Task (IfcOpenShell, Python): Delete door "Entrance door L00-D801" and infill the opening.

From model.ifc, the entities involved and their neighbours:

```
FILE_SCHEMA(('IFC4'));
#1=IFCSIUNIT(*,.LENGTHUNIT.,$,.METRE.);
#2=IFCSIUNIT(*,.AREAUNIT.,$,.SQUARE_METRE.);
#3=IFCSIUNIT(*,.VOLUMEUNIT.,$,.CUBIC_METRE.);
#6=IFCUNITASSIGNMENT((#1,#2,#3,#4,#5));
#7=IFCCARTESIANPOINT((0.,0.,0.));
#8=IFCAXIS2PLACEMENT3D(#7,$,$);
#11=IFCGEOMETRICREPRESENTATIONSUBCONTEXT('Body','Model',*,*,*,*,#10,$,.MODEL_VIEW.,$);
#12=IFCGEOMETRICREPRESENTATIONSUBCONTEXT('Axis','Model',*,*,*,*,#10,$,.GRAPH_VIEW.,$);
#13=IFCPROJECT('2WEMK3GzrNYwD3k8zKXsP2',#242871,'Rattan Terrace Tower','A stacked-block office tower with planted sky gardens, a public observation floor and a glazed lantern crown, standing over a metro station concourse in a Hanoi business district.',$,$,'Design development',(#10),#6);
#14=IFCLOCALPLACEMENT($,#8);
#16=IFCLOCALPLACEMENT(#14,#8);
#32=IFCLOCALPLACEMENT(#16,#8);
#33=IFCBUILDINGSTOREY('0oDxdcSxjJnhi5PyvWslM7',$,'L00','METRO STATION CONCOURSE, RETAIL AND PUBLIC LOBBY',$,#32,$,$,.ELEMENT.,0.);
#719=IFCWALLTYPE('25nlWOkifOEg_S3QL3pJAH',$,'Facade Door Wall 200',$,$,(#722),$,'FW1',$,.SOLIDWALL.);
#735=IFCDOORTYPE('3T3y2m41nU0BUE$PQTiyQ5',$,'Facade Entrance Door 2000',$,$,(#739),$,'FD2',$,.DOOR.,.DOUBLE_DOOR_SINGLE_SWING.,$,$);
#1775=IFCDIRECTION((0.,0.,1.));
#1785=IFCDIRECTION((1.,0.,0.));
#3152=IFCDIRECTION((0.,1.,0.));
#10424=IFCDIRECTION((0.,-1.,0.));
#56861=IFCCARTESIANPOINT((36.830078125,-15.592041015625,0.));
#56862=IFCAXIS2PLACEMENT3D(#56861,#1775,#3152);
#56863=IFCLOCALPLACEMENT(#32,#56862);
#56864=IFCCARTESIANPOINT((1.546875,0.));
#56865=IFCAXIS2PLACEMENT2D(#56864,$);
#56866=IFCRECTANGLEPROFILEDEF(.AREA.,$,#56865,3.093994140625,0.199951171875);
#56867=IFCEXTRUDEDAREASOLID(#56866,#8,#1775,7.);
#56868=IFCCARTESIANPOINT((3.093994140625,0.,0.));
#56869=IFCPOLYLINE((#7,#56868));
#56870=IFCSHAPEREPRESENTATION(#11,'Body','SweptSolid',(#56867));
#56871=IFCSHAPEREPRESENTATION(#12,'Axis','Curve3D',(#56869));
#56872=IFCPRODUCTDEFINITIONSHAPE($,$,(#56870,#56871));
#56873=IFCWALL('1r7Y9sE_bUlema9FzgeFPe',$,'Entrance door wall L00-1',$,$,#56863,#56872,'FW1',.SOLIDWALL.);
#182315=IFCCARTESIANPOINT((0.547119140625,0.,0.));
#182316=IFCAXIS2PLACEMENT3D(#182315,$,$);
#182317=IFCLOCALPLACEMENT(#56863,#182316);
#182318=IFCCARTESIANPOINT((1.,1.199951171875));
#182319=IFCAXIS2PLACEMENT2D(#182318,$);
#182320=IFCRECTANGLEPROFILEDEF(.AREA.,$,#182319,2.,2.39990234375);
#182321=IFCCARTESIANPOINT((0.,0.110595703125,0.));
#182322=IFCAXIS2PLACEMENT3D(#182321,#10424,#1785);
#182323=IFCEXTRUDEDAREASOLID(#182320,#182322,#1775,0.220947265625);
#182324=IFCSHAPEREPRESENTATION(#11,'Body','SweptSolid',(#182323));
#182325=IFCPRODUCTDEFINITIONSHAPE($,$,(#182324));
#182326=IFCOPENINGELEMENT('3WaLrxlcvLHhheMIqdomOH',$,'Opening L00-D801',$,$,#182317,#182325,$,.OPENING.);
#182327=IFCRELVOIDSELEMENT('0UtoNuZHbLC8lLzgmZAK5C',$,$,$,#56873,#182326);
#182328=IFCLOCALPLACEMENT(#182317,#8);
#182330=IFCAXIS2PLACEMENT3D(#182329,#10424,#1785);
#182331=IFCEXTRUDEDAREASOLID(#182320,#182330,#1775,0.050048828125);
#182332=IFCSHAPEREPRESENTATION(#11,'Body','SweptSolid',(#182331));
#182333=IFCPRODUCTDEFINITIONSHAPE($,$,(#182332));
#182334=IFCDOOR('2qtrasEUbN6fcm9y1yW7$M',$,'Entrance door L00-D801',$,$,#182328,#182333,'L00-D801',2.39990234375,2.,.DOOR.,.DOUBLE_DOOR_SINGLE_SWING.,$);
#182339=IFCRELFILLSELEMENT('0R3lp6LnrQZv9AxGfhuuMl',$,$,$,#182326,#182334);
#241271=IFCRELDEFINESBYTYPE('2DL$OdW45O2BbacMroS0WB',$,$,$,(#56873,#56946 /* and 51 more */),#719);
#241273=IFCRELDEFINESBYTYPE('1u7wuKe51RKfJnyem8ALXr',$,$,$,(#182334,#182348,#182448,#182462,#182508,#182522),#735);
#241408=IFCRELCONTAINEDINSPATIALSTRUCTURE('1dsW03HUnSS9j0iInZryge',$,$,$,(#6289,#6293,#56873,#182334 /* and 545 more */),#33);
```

```python
import ifcopenshell
import ifcopenshell.api.feature
import ifcopenshell.api.root
import ifcopenshell.geom
import ifcopenshell.util.shape

model = ifcopenshell.open("model.ifc")
settings = ifcopenshell.geom.settings()


def volume(element):
    """Net volume in cubic metres, openings subtracted."""
    shape = ifcopenshell.geom.create_shape(settings, element)
    return ifcopenshell.util.shape.get_volume(shape.geometry)


door = model.by_guid("2qtrasEUbN6fcm9y1yW7$M")
opening = door.FillsVoids[0].RelatingOpeningElement
wall = opening.VoidsElements[0].RelatingBuildingElement
before = volume(wall)

ifcopenshell.api.root.remove_product(model, product=door)
ifcopenshell.api.feature.remove_feature(model, feature=opening)

after = volume(wall)

print(f"wall volume {before:.3f} -> {after:.3f} m3")

model.write("model_updated.ifc")
```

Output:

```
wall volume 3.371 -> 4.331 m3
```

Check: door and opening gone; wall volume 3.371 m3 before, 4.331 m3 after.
